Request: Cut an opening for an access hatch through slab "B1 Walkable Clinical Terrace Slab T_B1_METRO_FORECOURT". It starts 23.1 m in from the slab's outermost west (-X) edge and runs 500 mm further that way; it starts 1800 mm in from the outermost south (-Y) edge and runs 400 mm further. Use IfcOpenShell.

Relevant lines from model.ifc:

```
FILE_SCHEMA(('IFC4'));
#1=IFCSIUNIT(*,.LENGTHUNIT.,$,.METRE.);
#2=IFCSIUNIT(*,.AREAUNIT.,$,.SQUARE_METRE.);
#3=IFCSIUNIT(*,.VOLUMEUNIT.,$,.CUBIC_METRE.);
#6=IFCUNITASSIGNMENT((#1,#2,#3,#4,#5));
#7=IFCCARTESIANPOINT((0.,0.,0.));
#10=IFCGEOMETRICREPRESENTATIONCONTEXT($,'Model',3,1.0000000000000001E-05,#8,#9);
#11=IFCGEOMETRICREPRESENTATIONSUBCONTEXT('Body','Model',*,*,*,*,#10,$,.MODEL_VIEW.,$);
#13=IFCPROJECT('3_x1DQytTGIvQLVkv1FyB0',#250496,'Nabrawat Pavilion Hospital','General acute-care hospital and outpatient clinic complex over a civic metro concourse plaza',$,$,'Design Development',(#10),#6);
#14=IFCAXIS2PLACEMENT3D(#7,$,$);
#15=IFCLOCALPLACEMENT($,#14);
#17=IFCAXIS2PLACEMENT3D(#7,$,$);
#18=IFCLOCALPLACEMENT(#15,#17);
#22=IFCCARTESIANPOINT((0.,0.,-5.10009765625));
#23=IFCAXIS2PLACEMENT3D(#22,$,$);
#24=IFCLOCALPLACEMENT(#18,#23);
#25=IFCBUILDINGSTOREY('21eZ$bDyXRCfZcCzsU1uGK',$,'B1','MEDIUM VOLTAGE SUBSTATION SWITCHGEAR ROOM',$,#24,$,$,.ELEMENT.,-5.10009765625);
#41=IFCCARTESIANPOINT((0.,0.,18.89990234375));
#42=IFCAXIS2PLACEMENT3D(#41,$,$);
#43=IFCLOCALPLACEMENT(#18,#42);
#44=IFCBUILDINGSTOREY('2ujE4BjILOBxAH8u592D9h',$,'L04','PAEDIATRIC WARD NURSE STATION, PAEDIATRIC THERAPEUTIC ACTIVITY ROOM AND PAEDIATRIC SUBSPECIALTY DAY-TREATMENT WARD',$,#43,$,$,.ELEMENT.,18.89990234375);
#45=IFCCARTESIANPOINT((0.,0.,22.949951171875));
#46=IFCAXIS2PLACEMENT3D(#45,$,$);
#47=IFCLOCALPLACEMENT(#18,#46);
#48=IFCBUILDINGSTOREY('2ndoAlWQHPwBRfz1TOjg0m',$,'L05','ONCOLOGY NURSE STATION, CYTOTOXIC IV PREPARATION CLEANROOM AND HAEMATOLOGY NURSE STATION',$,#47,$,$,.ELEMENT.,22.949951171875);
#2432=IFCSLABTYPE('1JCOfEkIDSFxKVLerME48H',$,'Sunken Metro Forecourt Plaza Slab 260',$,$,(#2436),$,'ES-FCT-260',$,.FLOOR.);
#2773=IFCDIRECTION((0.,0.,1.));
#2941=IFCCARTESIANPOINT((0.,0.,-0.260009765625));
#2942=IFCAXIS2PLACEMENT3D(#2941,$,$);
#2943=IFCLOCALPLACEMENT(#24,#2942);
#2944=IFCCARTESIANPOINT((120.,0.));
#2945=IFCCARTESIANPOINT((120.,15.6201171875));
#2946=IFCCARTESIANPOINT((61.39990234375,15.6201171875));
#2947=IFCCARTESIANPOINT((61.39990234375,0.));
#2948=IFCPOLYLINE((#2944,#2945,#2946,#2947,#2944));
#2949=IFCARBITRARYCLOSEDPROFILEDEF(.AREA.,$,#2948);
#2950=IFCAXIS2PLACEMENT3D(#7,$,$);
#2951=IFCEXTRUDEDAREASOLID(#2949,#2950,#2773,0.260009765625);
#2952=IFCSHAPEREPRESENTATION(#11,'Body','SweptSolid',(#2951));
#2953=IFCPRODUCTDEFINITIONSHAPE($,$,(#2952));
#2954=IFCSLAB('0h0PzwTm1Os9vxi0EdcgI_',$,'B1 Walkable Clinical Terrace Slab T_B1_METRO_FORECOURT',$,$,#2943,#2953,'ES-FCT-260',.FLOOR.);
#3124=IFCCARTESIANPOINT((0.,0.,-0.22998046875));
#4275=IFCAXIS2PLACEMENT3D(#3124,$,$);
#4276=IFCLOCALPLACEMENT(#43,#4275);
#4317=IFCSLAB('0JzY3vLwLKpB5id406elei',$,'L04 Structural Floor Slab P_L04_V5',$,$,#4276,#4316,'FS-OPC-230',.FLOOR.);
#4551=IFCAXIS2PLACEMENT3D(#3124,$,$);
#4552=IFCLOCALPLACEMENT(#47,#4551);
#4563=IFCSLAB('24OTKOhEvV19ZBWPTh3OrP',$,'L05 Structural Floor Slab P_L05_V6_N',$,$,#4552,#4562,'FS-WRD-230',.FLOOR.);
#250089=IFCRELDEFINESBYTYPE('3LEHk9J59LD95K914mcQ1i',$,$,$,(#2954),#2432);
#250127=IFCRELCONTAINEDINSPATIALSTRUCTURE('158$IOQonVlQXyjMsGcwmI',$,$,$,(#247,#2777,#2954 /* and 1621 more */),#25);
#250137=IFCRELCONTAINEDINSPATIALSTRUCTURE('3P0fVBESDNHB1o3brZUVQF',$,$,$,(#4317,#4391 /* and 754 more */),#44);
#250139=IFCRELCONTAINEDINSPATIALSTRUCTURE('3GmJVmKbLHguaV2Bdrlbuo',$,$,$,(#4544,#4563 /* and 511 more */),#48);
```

```python
import numpy as np
import ifcopenshell
import ifcopenshell.api.feature
import ifcopenshell.api.geometry
import ifcopenshell.api.root
import ifcopenshell.geom
import ifcopenshell.util.placement
import ifcopenshell.util.representation
import ifcopenshell.util.shape
import ifcopenshell.util.unit

model = ifcopenshell.open("model.ifc")
unit_scale = ifcopenshell.util.unit.calculate_unit_scale(model)
settings = ifcopenshell.geom.settings()


def volume(element):
    """Net volume in cubic metres, openings subtracted."""
    shape = ifcopenshell.geom.create_shape(settings, element)
    return ifcopenshell.util.shape.get_volume(shape.geometry)


slab = model.by_id(2954)
before = volume(slab)

# Extent in the slab's own axes, in metres. The edges named are its -X and -Y sides.
slab_shape = ifcopenshell.geom.create_shape(settings, slab)
vertices = ifcopenshell.util.shape.get_vertices(slab_shape.geometry)
x_min, y_min, bottom = vertices.min(axis=0)
top = vertices[:, 2].max()

opening = ifcopenshell.api.root.create_entity(model, ifc_class="IfcOpeningElement", name="Access hatch opening", predefined_type="OPENING")
context = ifcopenshell.util.representation.get_context(model, "Model", "Body", "MODEL_VIEW")
width, depth = 0.5, 0.4
outline = [(0.0, 0.0), (width, 0.0), (width, depth), (0.0, depth), (0.0, 0.0)]
# Overshoot both faces by 50 mm so the cut is clean.
shape = ifcopenshell.api.geometry.add_slab_representation(
    model, context=context, depth=top - bottom + 0.1, polyline=outline
)
ifcopenshell.api.geometry.assign_representation(model, product=opening, representation=shape)

matrix = ifcopenshell.util.placement.get_local_placement(slab.ObjectPlacement)
matrix[:, 3] = matrix @ np.append(np.array([x_min + 23.1, y_min + 1.8, bottom - 0.05]) / unit_scale, 1.0)
ifcopenshell.api.geometry.edit_object_placement(model, product=opening, matrix=matrix, is_si=False)
ifcopenshell.api.feature.add_feature(model, feature=opening, element=slab)

after = volume(slab)

print(f"slab volume {before:.3f} -> {after:.3f} m3")

model.write("model_rev.ifc")
```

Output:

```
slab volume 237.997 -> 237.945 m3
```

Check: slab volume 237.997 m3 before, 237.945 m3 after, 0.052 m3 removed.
